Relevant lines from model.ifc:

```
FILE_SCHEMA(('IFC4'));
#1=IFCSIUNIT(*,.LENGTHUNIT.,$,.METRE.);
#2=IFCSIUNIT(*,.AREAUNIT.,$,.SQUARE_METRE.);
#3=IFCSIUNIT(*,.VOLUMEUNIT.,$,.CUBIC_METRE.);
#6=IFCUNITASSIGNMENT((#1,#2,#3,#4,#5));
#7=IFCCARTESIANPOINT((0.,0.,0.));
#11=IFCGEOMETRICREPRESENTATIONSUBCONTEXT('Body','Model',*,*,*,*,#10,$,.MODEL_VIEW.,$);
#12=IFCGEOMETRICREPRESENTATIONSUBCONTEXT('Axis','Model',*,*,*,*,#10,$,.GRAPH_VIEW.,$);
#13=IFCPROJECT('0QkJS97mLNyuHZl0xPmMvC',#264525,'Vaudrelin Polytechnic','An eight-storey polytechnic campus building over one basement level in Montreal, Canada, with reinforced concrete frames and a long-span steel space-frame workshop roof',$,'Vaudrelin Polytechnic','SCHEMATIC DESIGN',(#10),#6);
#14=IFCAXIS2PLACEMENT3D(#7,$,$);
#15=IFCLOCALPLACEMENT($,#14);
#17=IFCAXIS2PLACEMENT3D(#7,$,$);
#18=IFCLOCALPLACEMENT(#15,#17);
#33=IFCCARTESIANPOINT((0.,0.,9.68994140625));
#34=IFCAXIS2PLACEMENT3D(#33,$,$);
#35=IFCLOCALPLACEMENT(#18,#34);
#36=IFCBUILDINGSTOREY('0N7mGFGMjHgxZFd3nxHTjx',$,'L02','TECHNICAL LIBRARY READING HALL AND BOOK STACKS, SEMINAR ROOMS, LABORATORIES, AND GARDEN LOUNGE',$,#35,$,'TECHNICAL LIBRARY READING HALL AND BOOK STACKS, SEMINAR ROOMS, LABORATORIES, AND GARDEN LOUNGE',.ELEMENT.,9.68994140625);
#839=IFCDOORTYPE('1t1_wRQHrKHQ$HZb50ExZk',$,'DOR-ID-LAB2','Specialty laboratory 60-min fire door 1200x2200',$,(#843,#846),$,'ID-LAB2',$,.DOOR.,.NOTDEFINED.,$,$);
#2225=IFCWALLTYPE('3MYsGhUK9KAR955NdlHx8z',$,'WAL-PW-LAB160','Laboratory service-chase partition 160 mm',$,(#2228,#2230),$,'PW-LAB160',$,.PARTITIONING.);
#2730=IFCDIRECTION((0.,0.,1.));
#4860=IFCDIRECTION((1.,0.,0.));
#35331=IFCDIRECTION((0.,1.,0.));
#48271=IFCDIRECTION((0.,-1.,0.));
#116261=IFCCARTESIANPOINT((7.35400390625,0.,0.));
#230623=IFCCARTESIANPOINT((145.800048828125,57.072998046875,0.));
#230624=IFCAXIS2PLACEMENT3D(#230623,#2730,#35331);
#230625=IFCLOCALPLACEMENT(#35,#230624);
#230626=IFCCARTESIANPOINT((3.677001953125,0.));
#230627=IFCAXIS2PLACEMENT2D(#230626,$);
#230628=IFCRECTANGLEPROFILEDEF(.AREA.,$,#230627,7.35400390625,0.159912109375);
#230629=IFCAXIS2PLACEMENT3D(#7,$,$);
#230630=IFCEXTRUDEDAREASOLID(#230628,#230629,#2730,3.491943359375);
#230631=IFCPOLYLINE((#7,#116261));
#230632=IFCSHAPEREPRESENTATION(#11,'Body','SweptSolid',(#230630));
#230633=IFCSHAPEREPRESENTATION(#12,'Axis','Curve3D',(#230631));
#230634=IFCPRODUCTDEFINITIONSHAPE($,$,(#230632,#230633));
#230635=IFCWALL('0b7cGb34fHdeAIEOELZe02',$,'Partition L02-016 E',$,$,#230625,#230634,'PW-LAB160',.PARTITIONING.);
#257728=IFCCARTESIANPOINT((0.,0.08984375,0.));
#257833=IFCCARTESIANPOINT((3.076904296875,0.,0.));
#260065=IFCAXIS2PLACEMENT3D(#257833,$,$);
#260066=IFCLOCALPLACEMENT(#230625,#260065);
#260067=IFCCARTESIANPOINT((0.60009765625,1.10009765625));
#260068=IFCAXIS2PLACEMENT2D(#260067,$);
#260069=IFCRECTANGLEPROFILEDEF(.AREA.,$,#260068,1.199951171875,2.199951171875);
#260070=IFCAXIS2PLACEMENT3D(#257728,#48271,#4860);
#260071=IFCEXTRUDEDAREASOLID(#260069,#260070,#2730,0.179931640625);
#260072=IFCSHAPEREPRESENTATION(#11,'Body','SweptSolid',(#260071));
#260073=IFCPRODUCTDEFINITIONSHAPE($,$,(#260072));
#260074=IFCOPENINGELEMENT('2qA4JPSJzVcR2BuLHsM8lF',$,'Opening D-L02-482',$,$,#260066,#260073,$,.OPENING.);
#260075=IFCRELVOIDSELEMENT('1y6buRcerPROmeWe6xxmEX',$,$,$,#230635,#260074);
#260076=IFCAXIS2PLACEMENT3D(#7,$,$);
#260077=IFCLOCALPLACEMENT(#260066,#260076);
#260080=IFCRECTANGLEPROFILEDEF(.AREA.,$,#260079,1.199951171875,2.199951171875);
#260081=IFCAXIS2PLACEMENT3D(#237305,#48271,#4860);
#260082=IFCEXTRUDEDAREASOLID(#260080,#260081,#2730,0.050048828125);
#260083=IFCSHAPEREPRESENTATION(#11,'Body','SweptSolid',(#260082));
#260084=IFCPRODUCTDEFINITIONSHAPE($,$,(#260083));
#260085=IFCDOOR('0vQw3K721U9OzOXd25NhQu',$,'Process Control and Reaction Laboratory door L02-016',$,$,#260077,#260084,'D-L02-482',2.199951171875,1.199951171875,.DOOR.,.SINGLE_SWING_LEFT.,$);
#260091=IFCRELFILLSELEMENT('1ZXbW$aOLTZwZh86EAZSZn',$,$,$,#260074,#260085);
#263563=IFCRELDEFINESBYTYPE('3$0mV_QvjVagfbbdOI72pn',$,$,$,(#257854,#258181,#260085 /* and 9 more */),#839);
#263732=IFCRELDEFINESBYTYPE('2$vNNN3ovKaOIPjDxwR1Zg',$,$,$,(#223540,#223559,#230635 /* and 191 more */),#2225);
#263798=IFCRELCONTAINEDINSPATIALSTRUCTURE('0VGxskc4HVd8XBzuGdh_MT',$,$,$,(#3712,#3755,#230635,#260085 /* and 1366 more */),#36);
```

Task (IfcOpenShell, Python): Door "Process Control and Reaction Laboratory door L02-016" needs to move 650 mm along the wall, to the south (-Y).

```python
import ifcopenshell
import ifcopenshell.api.geometry
import ifcopenshell.util.placement

model = ifcopenshell.open("model.ifc")

door = model.by_id(260085)
opening = door.FillsVoids[0].RelatingOpeningElement
wall = opening.VoidsElements[0].RelatingBuildingElement

wall_matrix = ifcopenshell.util.placement.get_local_placement(wall.ObjectPlacement)
shift = wall_matrix[:3, 0] * -0.65
before = ifcopenshell.util.placement.get_local_placement(door.ObjectPlacement)[:3, 3].copy()

# The door is placed relative to its opening, so it follows when the opening moves.
matrix = ifcopenshell.util.placement.get_local_placement(opening.ObjectPlacement)
matrix[:3, 3] += shift
ifcopenshell.api.geometry.edit_object_placement(
    model, product=opening, matrix=matrix, is_si=False, should_transform_children=True
)

after = ifcopenshell.util.placement.get_local_placement(door.ObjectPlacement)[:3, 3]
print("door moved by", (after - before).round(3) + 0.0)

model.write("model_updated.ifc")
```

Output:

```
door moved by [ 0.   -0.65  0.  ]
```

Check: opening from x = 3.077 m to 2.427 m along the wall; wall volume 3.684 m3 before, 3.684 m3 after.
